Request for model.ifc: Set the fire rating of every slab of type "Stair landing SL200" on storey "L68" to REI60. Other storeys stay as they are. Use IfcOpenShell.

First a look at what the model holds.

```python
import ifcopenshell
import ifcopenshell.util.element

model = ifcopenshell.open("model.ifc")
print(model.schema)
storey = next(s for s in model.by_type("IfcBuildingStorey") if s.Name == "L68")
slabs = [e for e in ifcopenshell.util.element.get_decomposition(storey) if e.is_a("IfcSlab")]
seen = {}
for e in slabs:
    element_type = ifcopenshell.util.element.get_type(e)
    key = (element_type.Name if element_type != e and element_type else None, ifcopenshell.util.element.get_pset(e, "Pset_SlabCommon", "FireRating"))
    seen[key] = seen.get(key, 0) + 1
for (name, value), count in sorted(seen.items(), key=str):
    print(count, "x", name, "|", value)
```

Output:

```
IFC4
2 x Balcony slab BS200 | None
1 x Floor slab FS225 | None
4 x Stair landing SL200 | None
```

```python
import ifcopenshell
import ifcopenshell.api.pset
import ifcopenshell.util.element

model = ifcopenshell.open("model.ifc")

storey = next(s for s in model.by_type("IfcBuildingStorey") if s.Name == "L68")
slabs = [e for e in ifcopenshell.util.element.get_decomposition(storey) if e.is_a("IfcSlab")]

count = 0
for e in slabs:
    element_type = ifcopenshell.util.element.get_type(e)
    if element_type in (None, e) or element_type.Name != "Stair landing SL200":
        continue
    found = ifcopenshell.util.element.get_pset(e, "Pset_SlabCommon", should_inherit=False)
    if found:
        pset = model.by_id(found["id"])
        if len(ifcopenshell.util.element.get_elements_by_pset(pset)) > 1:
            pset = ifcopenshell.api.pset.unshare_pset(model, products=[e], pset=pset)[0]
    else:
        pset = ifcopenshell.api.pset.add_pset(model, product=e, name="Pset_SlabCommon")
    ifcopenshell.api.pset.edit_pset(model, pset=pset, properties={"FireRating": "REI60"})
    count += 1

print(count, "slabs updated")

model.write("model_updated.ifc")
```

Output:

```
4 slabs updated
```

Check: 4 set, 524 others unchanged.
